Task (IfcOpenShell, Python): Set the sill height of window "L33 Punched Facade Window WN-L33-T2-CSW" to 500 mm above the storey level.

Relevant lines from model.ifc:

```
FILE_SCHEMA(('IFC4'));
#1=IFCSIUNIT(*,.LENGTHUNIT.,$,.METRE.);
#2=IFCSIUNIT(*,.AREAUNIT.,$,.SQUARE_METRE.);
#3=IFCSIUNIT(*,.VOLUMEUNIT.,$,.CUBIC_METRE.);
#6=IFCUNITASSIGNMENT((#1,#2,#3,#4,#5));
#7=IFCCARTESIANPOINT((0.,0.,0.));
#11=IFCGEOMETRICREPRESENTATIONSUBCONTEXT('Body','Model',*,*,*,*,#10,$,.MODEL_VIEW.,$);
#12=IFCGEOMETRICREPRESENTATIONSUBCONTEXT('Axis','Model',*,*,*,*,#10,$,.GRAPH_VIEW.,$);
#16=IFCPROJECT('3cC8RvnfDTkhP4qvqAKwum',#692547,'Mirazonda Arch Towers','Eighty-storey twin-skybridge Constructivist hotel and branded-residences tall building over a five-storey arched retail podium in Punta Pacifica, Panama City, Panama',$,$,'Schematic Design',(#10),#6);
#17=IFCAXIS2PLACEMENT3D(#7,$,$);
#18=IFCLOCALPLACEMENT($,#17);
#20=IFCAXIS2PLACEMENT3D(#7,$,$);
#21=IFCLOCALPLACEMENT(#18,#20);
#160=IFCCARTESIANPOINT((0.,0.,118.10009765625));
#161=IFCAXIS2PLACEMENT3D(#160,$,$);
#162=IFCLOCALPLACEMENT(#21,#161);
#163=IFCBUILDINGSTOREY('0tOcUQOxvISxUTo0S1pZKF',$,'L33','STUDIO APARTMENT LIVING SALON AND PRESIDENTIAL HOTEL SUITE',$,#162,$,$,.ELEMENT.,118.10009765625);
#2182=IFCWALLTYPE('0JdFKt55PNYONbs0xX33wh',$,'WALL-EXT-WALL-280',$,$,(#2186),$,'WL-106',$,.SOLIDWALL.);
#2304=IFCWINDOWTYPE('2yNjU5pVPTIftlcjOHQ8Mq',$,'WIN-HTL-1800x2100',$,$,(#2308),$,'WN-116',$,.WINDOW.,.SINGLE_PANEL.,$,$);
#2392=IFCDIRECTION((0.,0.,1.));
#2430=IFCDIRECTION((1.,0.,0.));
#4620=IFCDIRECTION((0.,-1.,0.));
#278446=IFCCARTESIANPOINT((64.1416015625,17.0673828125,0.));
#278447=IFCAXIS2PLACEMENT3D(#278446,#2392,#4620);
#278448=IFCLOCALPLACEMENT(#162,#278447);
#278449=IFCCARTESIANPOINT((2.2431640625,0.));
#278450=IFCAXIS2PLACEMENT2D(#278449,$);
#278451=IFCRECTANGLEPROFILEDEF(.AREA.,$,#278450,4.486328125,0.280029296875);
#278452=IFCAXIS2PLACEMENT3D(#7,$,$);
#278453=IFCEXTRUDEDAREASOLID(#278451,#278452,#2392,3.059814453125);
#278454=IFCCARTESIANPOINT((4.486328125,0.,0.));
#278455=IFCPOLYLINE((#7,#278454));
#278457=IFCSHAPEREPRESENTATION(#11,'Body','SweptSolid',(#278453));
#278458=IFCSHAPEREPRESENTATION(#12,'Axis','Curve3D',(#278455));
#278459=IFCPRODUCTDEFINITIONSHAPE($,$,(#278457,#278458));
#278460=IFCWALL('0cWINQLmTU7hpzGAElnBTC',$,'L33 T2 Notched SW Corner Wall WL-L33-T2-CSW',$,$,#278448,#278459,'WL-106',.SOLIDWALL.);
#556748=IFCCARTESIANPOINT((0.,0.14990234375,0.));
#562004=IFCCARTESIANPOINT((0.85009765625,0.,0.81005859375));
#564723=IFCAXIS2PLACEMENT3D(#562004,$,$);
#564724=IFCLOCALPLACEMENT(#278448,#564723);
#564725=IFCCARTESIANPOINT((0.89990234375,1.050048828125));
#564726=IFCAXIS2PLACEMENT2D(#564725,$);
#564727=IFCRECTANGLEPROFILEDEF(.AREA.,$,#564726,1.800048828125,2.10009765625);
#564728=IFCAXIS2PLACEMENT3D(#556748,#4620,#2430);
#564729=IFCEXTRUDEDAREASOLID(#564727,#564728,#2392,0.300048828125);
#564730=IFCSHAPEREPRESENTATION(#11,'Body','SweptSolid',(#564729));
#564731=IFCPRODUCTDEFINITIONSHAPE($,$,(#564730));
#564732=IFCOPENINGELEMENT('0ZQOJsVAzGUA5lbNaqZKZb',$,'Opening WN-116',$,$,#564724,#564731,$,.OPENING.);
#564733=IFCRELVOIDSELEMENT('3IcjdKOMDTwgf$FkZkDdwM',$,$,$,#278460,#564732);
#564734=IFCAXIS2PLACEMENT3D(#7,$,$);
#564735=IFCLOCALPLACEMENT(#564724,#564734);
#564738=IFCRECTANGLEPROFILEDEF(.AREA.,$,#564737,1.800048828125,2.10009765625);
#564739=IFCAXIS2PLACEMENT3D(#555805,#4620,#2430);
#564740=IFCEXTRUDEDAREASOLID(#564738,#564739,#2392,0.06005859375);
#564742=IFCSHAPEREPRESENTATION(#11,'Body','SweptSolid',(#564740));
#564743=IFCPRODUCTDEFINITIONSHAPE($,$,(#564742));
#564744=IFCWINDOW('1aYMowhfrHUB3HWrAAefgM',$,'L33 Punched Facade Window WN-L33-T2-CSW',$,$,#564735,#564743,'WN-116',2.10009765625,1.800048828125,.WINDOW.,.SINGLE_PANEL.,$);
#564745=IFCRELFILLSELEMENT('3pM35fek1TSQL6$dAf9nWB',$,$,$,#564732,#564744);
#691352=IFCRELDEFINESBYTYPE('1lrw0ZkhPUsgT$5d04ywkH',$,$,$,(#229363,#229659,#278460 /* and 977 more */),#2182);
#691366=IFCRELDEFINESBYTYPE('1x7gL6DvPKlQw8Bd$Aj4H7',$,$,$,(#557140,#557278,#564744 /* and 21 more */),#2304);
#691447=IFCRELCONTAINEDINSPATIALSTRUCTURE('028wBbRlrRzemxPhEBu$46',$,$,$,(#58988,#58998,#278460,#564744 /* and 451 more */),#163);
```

```python
import numpy as np
import ifcopenshell
import ifcopenshell.api.geometry
import ifcopenshell.geom
import ifcopenshell.util.element
import ifcopenshell.util.placement
import ifcopenshell.util.shape
import ifcopenshell.util.unit

model = ifcopenshell.open("model.ifc")
unit_scale = ifcopenshell.util.unit.calculate_unit_scale(model)

window = model.by_guid("1aYMowhfrHUB3HWrAAefgM")
opening = window.FillsVoids[0].RelatingOpeningElement
storey = ifcopenshell.util.element.get_container(window, ifc_class="IfcBuildingStorey")
level = ifcopenshell.util.placement.get_local_placement(storey.ObjectPlacement)[2, 3]

# The opening's origin need not be at the sill, so measure its lowest point.
shape = ifcopenshell.geom.create_shape(ifcopenshell.geom.settings(), opening)
bottom = ifcopenshell.util.shape.get_shape_bottom_elevation(shape, shape.geometry) / unit_scale
dz = level + 0.5 - bottom

shift = np.array([0.0, 0.0, dz])
# The window is placed relative to its opening, so it follows when the opening moves.
matrix = ifcopenshell.util.placement.get_local_placement(opening.ObjectPlacement)
matrix[:3, 3] += shift
ifcopenshell.api.geometry.edit_object_placement(
    model, product=opening, matrix=matrix, is_si=False, should_transform_children=True
)

print(f"moved by {dz * unit_scale:+.3f} m")

model.write("model_v2.ifc")
```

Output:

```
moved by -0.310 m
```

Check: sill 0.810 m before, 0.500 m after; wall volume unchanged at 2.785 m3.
